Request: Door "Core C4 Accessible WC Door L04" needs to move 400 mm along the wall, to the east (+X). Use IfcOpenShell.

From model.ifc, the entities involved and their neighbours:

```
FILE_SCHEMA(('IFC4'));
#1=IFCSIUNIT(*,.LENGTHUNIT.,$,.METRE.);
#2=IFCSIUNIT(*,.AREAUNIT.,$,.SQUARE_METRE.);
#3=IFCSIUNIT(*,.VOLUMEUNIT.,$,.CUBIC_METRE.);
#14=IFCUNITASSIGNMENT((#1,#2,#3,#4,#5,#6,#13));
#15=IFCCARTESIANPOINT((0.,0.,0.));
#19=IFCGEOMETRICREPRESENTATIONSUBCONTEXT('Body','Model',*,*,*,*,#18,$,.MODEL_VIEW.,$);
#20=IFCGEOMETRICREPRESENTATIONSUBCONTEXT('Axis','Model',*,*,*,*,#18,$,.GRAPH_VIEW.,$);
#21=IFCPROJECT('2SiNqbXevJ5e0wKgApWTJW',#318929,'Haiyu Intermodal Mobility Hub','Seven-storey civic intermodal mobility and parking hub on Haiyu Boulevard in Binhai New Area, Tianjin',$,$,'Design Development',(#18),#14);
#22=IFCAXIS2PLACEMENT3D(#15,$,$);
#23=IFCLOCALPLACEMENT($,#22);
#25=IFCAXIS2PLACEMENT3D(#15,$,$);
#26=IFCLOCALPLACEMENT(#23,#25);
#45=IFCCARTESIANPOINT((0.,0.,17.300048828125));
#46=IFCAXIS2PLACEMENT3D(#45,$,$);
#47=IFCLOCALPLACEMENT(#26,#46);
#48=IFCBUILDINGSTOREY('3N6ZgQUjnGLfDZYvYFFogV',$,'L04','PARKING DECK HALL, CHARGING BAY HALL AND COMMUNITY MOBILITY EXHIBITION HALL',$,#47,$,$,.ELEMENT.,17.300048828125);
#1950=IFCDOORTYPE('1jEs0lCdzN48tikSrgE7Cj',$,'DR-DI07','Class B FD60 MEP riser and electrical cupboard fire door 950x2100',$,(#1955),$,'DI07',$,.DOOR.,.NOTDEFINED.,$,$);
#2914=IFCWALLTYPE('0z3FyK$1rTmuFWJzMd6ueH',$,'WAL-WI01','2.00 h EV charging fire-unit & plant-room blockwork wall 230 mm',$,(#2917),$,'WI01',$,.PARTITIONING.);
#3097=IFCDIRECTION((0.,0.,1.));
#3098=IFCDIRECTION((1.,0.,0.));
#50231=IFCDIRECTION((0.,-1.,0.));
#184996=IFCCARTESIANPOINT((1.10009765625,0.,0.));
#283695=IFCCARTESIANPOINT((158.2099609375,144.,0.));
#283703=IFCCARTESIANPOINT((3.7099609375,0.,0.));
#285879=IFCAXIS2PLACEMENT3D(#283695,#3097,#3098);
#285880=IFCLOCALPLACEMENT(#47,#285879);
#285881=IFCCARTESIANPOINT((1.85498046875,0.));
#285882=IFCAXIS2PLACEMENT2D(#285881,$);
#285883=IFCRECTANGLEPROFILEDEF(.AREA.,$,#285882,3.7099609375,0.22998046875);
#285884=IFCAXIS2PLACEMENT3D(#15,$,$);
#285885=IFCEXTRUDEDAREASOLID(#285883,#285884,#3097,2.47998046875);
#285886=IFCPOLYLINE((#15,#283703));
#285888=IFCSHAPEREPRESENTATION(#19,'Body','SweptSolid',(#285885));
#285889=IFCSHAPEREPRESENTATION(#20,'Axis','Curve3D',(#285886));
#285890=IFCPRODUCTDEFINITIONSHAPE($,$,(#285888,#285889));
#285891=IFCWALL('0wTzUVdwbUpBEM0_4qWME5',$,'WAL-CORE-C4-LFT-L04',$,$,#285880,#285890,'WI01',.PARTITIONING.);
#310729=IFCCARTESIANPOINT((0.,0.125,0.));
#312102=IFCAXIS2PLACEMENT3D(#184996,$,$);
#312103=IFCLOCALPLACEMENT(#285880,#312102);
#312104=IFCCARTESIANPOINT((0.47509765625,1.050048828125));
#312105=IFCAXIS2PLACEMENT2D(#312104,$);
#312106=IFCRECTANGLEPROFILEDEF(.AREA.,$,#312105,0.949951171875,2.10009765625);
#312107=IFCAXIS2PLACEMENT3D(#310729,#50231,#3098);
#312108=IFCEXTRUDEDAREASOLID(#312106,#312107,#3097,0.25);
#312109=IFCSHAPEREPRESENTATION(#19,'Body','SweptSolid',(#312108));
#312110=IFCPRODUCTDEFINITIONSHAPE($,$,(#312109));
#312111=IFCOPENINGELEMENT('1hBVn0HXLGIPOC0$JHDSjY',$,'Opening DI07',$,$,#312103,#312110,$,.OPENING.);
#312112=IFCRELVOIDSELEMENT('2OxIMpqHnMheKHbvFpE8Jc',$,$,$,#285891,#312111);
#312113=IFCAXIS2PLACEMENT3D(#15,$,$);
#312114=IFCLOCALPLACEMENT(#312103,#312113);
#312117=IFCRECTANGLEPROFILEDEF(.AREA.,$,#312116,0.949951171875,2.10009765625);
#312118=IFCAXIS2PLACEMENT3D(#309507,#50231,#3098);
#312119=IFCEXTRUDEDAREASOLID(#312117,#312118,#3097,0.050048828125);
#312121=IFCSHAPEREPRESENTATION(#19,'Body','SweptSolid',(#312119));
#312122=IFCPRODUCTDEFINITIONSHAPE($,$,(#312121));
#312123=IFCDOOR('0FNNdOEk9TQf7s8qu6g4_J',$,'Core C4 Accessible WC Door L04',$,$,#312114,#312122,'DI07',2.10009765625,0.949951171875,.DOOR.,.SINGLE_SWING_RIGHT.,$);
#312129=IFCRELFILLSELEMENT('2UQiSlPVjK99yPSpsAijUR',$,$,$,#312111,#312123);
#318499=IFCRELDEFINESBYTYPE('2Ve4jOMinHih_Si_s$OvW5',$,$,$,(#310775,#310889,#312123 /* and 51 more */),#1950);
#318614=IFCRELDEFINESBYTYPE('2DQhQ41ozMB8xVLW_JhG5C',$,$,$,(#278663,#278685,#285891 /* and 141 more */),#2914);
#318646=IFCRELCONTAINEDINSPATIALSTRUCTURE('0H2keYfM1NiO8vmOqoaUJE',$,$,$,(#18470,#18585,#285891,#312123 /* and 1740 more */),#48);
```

```python
import ifcopenshell
import ifcopenshell.api.geometry
import ifcopenshell.util.placement
import ifcopenshell.util.unit

model = ifcopenshell.open("model.ifc")
unit_scale = ifcopenshell.util.unit.calculate_unit_scale(model)

door = model.by_id(312123)
opening = door.FillsVoids[0].RelatingOpeningElement
wall = opening.VoidsElements[0].RelatingBuildingElement

wall_matrix = ifcopenshell.util.placement.get_local_placement(wall.ObjectPlacement)
shift = wall_matrix[:3, 0] * 0.4 / unit_scale
before = ifcopenshell.util.placement.get_local_placement(door.ObjectPlacement)[:3, 3].copy()

# The door is placed relative to its opening, so it follows when the opening moves.
matrix = ifcopenshell.util.placement.get_local_placement(opening.ObjectPlacement)
matrix[:3, 3] += shift
ifcopenshell.api.geometry.edit_object_placement(
    model, product=opening, matrix=matrix, is_si=False, should_transform_children=True
)

after = ifcopenshell.util.placement.get_local_placement(door.ObjectPlacement)[:3, 3]
print("door moved by", (after - before).round(3) + 0.0)

model.write("model_rev.ifc")
```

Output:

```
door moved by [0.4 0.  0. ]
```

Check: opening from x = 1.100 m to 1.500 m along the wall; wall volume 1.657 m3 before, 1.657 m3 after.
